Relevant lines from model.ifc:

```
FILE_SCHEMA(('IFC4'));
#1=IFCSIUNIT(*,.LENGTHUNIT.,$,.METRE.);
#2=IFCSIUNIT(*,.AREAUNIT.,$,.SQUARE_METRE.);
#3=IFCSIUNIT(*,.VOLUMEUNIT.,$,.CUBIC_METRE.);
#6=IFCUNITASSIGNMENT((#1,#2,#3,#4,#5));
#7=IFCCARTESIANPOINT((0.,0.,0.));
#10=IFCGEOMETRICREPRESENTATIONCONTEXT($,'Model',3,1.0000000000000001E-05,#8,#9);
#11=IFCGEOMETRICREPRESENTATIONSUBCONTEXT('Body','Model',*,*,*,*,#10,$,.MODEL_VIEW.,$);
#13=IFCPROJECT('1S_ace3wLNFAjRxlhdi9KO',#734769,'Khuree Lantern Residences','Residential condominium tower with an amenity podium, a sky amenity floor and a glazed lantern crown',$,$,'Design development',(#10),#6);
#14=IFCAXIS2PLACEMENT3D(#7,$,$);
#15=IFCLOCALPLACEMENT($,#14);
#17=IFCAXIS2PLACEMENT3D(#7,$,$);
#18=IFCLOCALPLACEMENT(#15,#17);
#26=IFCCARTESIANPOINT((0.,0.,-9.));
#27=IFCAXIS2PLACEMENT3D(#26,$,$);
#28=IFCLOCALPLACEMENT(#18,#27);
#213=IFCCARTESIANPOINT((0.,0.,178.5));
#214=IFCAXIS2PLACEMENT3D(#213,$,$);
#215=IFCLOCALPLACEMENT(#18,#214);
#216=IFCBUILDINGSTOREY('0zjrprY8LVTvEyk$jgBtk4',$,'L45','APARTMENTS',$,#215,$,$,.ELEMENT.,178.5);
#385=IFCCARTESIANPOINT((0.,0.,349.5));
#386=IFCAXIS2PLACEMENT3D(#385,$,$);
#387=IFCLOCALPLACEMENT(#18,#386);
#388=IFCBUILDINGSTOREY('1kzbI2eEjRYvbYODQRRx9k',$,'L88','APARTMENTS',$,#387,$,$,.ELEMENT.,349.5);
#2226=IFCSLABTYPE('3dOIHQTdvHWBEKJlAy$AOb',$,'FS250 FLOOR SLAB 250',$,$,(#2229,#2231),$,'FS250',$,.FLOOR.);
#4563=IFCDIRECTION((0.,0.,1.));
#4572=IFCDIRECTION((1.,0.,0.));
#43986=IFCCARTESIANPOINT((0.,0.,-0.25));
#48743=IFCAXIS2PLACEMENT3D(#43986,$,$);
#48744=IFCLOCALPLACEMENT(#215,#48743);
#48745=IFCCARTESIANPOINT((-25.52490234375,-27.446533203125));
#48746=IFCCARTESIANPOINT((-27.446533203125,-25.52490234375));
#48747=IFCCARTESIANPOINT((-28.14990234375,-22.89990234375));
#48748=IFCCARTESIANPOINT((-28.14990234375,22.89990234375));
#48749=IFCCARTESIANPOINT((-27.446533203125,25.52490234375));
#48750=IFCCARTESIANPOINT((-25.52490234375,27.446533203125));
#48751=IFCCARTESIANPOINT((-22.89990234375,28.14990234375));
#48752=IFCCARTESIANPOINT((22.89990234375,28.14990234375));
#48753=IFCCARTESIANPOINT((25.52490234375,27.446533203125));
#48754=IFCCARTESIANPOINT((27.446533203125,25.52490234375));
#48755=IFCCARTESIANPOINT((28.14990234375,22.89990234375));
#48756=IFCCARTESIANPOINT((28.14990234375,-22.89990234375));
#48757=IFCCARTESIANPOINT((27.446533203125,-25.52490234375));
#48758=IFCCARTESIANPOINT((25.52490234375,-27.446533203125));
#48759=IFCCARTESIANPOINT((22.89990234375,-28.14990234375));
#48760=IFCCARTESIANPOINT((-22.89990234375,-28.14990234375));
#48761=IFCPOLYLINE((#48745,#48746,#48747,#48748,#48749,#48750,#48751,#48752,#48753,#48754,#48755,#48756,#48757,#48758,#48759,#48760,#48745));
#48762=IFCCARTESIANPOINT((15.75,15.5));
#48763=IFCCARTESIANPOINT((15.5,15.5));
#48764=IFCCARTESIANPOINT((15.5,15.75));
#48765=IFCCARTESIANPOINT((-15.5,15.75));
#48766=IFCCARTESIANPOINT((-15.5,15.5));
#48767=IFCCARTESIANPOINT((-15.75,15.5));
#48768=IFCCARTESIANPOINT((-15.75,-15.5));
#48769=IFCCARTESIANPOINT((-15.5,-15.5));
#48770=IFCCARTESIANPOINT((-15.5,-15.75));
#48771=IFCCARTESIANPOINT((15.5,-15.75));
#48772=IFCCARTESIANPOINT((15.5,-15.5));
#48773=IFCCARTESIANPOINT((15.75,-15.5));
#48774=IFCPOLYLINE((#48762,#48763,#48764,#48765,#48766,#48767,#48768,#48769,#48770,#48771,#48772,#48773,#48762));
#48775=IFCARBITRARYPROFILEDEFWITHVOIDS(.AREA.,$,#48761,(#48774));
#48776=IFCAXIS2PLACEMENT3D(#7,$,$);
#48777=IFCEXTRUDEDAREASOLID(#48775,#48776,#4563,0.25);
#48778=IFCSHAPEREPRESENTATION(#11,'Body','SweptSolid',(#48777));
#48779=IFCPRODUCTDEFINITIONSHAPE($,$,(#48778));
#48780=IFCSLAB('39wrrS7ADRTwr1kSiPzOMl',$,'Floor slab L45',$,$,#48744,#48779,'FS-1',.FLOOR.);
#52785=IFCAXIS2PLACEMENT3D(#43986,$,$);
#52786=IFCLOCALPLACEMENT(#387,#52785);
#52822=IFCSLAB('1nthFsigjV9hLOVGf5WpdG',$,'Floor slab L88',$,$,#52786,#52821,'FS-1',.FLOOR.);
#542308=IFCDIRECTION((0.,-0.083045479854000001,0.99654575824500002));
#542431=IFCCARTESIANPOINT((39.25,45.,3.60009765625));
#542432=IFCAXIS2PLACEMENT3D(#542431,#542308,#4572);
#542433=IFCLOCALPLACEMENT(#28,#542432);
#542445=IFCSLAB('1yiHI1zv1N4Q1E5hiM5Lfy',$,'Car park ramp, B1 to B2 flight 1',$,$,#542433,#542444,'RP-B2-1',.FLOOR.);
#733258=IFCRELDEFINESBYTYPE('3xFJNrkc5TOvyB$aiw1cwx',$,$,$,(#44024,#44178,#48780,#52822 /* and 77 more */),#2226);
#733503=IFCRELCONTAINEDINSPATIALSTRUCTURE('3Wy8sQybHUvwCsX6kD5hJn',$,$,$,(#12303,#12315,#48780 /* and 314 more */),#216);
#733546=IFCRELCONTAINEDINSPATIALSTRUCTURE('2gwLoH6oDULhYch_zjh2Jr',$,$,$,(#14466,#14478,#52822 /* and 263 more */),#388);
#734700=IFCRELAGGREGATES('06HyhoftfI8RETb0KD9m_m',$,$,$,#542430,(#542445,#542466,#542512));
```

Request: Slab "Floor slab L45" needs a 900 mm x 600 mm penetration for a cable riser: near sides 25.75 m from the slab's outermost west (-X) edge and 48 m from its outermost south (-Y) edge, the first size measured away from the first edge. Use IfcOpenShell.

```python
import numpy as np
import ifcopenshell
import ifcopenshell.api.feature
import ifcopenshell.api.geometry
import ifcopenshell.api.root
import ifcopenshell.geom
import ifcopenshell.util.placement
import ifcopenshell.util.representation
import ifcopenshell.util.shape
import ifcopenshell.util.unit

model = ifcopenshell.open("model.ifc")
unit_scale = ifcopenshell.util.unit.calculate_unit_scale(model)
settings = ifcopenshell.geom.settings()


def volume(element):
    """Net volume in cubic metres, openings subtracted."""
    shape = ifcopenshell.geom.create_shape(settings, element)
    return ifcopenshell.util.shape.get_volume(shape.geometry)


slab = model.by_guid("39wrrS7ADRTwr1kSiPzOMl")
before = volume(slab)

# Extent in the slab's own axes, in metres. The edges named are its -X and -Y sides.
slab_shape = ifcopenshell.geom.create_shape(settings, slab)
vertices = ifcopenshell.util.shape.get_vertices(slab_shape.geometry)
x_min, y_min, bottom = vertices.min(axis=0)
top = vertices[:, 2].max()

opening = ifcopenshell.api.root.create_entity(model, ifc_class="IfcOpeningElement", name="Cable riser opening", predefined_type="OPENING")
context = ifcopenshell.util.representation.get_context(model, "Model", "Body", "MODEL_VIEW")
width, depth = 0.9, 0.6
outline = [(0.0, 0.0), (width, 0.0), (width, depth), (0.0, depth), (0.0, 0.0)]
# Overshoot both faces by 50 mm so the cut is clean.
shape = ifcopenshell.api.geometry.add_slab_representation(
    model, context=context, depth=top - bottom + 0.1, polyline=outline
)
ifcopenshell.api.geometry.assign_representation(model, product=opening, representation=shape)

matrix = ifcopenshell.util.placement.get_local_placement(slab.ObjectPlacement)
matrix[:, 3] = matrix @ np.append(np.array([x_min + 25.75, y_min + 48, bottom - 0.05]) / unit_scale, 1.0)
ifcopenshell.api.geometry.edit_object_placement(model, product=opening, matrix=matrix, is_si=False)
ifcopenshell.api.feature.add_feature(model, feature=opening, element=slab)

after = volume(slab)

print(f"slab volume {before:.3f} -> {after:.3f} m3")

model.write("model_v2.ifc")
```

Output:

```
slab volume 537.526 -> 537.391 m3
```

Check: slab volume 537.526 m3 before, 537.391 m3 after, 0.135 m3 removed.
